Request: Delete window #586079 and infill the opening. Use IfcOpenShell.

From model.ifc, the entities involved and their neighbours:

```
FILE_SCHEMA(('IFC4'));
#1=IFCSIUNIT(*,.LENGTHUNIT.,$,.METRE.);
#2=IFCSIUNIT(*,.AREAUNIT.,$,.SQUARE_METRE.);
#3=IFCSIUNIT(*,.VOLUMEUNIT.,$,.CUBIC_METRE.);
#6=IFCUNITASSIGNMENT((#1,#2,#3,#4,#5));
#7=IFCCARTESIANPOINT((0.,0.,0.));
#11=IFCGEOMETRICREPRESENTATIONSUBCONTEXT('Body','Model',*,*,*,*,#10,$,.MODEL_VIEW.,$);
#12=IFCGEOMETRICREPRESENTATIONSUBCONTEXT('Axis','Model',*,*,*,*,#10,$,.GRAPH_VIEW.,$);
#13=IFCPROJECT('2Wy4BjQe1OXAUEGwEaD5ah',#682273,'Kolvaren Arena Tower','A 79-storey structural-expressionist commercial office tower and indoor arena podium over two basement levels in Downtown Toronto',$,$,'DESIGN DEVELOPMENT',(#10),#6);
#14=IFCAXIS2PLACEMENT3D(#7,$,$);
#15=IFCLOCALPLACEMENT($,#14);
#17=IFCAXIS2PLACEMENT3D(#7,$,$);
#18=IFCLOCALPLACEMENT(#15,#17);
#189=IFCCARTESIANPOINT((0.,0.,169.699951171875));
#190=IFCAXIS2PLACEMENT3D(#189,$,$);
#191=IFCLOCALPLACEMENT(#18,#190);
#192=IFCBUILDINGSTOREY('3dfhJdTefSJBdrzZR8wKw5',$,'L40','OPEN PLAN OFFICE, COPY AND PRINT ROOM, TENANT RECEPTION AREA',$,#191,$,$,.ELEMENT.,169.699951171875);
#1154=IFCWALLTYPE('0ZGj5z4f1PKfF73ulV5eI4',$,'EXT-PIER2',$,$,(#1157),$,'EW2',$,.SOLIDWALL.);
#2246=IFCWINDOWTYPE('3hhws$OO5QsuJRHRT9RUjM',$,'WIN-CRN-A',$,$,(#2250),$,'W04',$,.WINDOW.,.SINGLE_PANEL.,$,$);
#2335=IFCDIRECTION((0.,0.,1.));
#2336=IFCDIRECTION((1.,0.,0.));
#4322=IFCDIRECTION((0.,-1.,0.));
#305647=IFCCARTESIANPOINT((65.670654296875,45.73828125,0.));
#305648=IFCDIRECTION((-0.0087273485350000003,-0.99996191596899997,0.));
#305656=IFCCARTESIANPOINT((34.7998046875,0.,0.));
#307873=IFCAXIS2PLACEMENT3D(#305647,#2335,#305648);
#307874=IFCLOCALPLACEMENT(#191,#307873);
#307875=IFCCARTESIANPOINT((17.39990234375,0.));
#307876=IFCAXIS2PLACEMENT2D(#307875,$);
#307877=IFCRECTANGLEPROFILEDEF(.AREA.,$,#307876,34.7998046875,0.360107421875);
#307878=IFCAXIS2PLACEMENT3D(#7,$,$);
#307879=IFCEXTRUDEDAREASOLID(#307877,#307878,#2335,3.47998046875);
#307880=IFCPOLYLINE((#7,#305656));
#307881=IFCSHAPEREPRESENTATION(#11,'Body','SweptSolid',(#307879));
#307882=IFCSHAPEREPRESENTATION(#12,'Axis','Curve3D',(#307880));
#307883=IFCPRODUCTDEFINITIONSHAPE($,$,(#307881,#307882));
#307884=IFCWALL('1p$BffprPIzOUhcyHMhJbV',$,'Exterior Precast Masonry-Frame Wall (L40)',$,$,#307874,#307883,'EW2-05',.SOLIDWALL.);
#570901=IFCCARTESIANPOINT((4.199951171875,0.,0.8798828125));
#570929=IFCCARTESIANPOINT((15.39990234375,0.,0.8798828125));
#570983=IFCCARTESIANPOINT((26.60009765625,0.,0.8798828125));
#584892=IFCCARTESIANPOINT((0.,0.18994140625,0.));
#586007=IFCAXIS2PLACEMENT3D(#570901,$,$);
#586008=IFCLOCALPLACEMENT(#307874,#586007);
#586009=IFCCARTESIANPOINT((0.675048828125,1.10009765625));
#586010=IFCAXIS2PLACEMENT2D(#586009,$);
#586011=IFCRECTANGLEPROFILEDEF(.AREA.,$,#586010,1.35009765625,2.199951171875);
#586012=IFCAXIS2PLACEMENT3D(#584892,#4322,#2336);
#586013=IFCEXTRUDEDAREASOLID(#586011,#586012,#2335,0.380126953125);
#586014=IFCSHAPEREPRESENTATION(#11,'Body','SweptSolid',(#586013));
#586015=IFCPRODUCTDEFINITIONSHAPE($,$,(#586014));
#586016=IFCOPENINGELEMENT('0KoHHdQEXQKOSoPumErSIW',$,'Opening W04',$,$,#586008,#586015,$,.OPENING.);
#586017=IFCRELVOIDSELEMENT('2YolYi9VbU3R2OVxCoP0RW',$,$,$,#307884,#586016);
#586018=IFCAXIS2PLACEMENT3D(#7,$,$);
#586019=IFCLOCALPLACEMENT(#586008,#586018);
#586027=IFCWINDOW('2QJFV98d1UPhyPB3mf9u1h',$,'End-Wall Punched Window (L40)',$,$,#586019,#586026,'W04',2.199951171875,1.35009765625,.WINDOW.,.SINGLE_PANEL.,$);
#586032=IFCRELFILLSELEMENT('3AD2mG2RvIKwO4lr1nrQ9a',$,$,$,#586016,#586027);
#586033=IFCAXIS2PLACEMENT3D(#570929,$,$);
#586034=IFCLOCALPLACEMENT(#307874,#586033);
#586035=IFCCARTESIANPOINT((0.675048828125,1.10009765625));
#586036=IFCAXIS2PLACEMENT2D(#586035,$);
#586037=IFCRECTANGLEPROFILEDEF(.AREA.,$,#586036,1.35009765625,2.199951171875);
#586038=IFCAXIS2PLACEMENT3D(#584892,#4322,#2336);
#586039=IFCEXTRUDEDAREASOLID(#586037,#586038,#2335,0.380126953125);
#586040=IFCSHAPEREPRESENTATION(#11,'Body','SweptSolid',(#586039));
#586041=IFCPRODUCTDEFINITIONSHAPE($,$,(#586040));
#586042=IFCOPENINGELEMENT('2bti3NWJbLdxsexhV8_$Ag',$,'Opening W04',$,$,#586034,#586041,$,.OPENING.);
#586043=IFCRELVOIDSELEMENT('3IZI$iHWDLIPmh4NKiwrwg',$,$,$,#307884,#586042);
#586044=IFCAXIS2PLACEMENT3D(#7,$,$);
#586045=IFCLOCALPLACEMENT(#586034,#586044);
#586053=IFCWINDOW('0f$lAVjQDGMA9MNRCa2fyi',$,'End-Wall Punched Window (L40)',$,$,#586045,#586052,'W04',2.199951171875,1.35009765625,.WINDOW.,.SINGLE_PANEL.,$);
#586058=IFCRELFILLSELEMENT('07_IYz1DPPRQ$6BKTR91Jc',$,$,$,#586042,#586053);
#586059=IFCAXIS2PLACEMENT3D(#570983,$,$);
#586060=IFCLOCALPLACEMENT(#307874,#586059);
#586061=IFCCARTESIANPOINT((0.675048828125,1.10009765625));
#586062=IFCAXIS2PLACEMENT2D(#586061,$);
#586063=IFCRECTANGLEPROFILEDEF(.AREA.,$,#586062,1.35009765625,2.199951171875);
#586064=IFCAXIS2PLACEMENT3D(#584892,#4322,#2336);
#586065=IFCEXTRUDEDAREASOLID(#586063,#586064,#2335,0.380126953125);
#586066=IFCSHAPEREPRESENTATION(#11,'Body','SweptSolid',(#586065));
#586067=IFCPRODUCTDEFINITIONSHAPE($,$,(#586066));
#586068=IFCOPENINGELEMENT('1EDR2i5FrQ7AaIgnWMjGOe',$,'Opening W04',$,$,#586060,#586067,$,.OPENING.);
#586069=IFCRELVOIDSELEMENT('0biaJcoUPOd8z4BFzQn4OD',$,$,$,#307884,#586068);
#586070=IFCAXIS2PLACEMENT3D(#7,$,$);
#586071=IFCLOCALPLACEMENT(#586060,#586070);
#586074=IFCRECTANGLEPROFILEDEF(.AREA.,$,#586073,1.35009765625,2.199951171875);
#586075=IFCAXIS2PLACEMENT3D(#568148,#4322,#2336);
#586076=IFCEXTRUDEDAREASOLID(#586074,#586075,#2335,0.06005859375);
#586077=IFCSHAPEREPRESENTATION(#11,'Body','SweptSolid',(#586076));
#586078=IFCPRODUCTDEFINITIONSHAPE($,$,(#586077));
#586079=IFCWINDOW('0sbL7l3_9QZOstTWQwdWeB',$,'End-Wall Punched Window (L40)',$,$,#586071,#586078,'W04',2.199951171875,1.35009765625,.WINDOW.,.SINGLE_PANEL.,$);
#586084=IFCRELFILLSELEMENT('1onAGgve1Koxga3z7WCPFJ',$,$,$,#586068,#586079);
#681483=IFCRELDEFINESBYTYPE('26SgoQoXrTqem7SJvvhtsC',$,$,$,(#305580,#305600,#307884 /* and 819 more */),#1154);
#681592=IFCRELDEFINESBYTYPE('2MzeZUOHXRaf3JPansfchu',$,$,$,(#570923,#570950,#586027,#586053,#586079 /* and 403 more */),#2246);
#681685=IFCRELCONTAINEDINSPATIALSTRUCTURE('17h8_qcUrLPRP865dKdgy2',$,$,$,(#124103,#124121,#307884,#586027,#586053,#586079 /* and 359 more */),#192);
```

```python
import ifcopenshell
import ifcopenshell.api.feature
import ifcopenshell.api.root
import ifcopenshell.geom
import ifcopenshell.util.shape

model = ifcopenshell.open("model.ifc")
settings = ifcopenshell.geom.settings()


def volume(element):
    """Net volume in cubic metres, openings subtracted."""
    shape = ifcopenshell.geom.create_shape(settings, element)
    return ifcopenshell.util.shape.get_volume(shape.geometry)


window = model.by_guid("0sbL7l3_9QZOstTWQwdWeB")
opening = window.FillsVoids[0].RelatingOpeningElement
wall = opening.VoidsElements[0].RelatingBuildingElement
before = volume(wall)

ifcopenshell.api.root.remove_product(model, product=window)
ifcopenshell.api.feature.remove_feature(model, feature=opening)

after = volume(wall)

print(f"wall volume {before:.3f} -> {after:.3f} m3")

model.write("model_rev.ifc")
```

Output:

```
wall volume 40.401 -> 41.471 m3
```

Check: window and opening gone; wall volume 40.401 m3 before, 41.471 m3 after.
